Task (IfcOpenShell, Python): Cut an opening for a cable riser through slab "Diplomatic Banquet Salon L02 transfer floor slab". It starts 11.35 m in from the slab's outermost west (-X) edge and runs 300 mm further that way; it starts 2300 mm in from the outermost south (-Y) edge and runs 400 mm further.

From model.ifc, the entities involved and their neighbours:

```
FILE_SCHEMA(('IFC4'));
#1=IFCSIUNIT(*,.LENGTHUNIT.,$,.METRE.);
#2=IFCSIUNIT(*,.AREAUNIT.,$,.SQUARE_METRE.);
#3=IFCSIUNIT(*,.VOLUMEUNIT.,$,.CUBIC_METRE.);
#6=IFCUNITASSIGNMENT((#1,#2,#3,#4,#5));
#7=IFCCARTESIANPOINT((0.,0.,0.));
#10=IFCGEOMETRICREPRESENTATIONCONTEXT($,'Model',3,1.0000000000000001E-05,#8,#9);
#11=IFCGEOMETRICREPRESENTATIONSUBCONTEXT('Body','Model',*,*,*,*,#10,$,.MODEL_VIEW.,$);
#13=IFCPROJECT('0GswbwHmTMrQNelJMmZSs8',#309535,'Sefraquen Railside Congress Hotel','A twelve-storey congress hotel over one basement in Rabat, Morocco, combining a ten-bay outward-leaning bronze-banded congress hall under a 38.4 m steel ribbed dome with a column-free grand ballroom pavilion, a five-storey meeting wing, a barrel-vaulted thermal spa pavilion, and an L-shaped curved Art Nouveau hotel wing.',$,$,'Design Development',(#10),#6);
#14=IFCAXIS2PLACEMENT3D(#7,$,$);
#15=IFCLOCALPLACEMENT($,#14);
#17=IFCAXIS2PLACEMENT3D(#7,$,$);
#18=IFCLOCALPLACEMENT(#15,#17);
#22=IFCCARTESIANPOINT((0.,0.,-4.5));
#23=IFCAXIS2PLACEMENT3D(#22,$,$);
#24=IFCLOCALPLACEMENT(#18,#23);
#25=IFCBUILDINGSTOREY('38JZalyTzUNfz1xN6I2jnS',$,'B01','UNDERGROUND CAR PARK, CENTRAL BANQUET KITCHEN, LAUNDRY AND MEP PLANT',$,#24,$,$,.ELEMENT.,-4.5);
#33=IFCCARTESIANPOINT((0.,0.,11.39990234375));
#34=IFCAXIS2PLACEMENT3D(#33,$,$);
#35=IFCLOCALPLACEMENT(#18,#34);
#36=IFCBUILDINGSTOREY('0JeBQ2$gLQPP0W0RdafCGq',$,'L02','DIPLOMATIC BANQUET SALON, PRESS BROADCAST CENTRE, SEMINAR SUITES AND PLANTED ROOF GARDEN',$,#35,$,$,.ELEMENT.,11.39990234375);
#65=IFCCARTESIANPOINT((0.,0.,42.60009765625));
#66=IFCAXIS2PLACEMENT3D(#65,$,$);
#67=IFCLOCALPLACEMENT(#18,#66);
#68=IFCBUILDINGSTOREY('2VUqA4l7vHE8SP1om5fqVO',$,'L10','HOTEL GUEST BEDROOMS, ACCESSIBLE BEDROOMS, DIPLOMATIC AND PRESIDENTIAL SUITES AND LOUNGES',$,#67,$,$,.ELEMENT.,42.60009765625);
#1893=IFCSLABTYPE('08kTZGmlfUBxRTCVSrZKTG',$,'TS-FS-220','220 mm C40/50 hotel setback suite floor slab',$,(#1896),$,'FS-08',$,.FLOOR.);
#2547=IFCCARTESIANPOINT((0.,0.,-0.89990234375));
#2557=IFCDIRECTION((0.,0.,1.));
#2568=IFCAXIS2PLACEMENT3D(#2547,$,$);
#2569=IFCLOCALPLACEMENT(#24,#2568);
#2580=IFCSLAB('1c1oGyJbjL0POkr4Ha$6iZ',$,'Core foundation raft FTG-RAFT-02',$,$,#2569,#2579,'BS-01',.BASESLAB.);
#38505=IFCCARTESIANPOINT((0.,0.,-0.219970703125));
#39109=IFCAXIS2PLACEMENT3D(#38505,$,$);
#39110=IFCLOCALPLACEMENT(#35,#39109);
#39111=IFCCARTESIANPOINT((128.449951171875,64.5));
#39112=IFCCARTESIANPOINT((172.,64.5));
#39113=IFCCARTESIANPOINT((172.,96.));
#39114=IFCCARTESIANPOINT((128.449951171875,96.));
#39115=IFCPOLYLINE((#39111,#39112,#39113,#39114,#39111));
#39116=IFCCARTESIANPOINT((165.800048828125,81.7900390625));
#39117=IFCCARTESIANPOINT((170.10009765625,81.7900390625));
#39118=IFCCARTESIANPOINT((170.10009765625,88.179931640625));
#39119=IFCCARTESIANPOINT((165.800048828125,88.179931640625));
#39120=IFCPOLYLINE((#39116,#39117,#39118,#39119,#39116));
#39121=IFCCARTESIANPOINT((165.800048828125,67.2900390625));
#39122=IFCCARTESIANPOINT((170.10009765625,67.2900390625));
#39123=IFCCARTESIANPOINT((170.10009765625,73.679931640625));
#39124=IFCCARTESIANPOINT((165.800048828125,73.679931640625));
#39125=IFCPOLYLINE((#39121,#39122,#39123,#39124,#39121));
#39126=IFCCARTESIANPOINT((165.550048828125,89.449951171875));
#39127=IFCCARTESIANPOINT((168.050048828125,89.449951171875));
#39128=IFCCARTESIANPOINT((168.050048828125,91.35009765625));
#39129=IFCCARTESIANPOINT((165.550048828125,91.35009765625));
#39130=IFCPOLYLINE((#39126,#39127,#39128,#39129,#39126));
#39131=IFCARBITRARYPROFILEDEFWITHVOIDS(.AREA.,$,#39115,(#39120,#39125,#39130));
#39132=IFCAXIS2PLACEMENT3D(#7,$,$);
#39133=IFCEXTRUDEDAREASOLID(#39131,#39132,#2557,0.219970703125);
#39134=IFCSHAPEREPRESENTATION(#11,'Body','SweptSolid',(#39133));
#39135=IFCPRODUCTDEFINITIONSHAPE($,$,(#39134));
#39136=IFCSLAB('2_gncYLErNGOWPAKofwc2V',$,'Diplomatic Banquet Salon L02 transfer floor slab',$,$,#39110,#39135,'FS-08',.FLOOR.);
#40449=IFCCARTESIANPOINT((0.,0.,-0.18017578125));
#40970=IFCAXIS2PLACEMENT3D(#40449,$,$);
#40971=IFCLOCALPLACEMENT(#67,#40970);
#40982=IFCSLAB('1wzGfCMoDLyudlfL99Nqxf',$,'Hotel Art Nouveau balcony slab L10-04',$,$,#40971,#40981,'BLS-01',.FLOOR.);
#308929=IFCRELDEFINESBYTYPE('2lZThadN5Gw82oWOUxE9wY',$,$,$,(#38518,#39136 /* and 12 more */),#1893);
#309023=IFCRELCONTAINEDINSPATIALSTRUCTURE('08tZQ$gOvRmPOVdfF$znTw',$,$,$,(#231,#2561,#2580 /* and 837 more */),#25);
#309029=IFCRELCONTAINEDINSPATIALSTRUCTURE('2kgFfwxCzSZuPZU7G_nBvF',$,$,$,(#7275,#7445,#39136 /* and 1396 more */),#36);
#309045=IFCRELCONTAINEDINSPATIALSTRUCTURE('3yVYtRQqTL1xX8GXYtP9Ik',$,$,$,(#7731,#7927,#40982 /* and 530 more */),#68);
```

```python
import numpy as np
import ifcopenshell
import ifcopenshell.api.feature
import ifcopenshell.api.geometry
import ifcopenshell.api.root
import ifcopenshell.geom
import ifcopenshell.util.placement
import ifcopenshell.util.representation
import ifcopenshell.util.shape
import ifcopenshell.util.unit

model = ifcopenshell.open("model.ifc")
unit_scale = ifcopenshell.util.unit.calculate_unit_scale(model)
settings = ifcopenshell.geom.settings()


def volume(element):
    """Net volume in cubic metres, openings subtracted."""
    shape = ifcopenshell.geom.create_shape(settings, element)
    return ifcopenshell.util.shape.get_volume(shape.geometry)


slab = model.by_guid("2_gncYLErNGOWPAKofwc2V")
before = volume(slab)

# Extent in the slab's own axes, in metres. The edges named are its -X and -Y sides.
slab_shape = ifcopenshell.geom.create_shape(settings, slab)
vertices = ifcopenshell.util.shape.get_vertices(slab_shape.geometry)
x_min, y_min, bottom = vertices.min(axis=0)
top = vertices[:, 2].max()

opening = ifcopenshell.api.root.create_entity(model, ifc_class="IfcOpeningElement", name="Cable riser opening", predefined_type="OPENING")
context = ifcopenshell.util.representation.get_context(model, "Model", "Body", "MODEL_VIEW")
width, depth = 0.3, 0.4
outline = [(0.0, 0.0), (width, 0.0), (width, depth), (0.0, depth), (0.0, 0.0)]
# Overshoot both faces by 50 mm so the cut is clean.
shape = ifcopenshell.api.geometry.add_slab_representation(
    model, context=context, depth=top - bottom + 0.1, polyline=outline
)
ifcopenshell.api.geometry.assign_representation(model, product=opening, representation=shape)

matrix = ifcopenshell.util.placement.get_local_placement(slab.ObjectPlacement)
matrix[:, 3] = matrix @ np.append(np.array([x_min + 11.35, y_min + 2.3, bottom - 0.05]) / unit_scale, 1.0)
ifcopenshell.api.geometry.edit_object_placement(model, product=opening, matrix=matrix, is_si=False)
ifcopenshell.api.feature.add_feature(model, feature=opening, element=slab)

after = volume(slab)

print(f"slab volume {before:.3f} -> {after:.3f} m3")

model.write("model-out.ifc")
```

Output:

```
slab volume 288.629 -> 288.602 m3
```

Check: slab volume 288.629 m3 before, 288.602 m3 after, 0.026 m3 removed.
